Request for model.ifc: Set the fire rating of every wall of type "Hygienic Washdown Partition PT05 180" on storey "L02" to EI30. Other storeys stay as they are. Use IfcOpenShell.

First a look at what the model holds.

```python
import ifcopenshell
import ifcopenshell.util.element

model = ifcopenshell.open("model.ifc")
print(model.schema)
storey = next(s for s in model.by_type("IfcBuildingStorey") if s.Name == "L02")
walls = [e for e in ifcopenshell.util.element.get_decomposition(storey) if e.is_a("IfcWall")]
seen = {}
for e in walls:
    element_type = ifcopenshell.util.element.get_type(e)
    key = (element_type.Name if element_type != e and element_type else None, ifcopenshell.util.element.get_pset(e, "Pset_WallCommon", "FireRating"))
    seen[key] = seen.get(key, 0) + 1
for (name, value), count in sorted(seen.items(), key=str):
    print(count, "x", name, "|", value)
```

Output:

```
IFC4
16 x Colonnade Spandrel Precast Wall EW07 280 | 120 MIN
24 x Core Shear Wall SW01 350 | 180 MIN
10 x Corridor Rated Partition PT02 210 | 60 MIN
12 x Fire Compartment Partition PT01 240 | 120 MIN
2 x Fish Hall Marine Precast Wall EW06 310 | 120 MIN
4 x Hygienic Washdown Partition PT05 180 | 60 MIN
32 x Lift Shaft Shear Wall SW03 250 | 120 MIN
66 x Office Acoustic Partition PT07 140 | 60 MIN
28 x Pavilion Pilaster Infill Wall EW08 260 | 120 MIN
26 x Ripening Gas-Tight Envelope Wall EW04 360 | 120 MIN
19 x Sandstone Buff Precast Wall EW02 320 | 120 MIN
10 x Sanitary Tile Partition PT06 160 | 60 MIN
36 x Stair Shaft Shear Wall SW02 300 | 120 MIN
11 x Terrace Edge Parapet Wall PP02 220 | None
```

```python
import ifcopenshell
import ifcopenshell.api.pset
import ifcopenshell.util.element

model = ifcopenshell.open("model.ifc")

storey = next(s for s in model.by_type("IfcBuildingStorey") if s.Name == "L02")
walls = [e for e in ifcopenshell.util.element.get_decomposition(storey) if e.is_a("IfcWall")]

count = 0
for e in walls:
    element_type = ifcopenshell.util.element.get_type(e)
    if element_type in (None, e) or element_type.Name != "Hygienic Washdown Partition PT05 180":
        continue
    # add_pset returns the element's existing set when there is one.
    pset = ifcopenshell.api.pset.add_pset(model, product=e, name="Pset_WallCommon")
    ifcopenshell.api.pset.edit_pset(model, pset=pset, properties={"FireRating": "EI30"})
    count += 1

print(count, "walls updated")

model.write("model_edited.ifc")
```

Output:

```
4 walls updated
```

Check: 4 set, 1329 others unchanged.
